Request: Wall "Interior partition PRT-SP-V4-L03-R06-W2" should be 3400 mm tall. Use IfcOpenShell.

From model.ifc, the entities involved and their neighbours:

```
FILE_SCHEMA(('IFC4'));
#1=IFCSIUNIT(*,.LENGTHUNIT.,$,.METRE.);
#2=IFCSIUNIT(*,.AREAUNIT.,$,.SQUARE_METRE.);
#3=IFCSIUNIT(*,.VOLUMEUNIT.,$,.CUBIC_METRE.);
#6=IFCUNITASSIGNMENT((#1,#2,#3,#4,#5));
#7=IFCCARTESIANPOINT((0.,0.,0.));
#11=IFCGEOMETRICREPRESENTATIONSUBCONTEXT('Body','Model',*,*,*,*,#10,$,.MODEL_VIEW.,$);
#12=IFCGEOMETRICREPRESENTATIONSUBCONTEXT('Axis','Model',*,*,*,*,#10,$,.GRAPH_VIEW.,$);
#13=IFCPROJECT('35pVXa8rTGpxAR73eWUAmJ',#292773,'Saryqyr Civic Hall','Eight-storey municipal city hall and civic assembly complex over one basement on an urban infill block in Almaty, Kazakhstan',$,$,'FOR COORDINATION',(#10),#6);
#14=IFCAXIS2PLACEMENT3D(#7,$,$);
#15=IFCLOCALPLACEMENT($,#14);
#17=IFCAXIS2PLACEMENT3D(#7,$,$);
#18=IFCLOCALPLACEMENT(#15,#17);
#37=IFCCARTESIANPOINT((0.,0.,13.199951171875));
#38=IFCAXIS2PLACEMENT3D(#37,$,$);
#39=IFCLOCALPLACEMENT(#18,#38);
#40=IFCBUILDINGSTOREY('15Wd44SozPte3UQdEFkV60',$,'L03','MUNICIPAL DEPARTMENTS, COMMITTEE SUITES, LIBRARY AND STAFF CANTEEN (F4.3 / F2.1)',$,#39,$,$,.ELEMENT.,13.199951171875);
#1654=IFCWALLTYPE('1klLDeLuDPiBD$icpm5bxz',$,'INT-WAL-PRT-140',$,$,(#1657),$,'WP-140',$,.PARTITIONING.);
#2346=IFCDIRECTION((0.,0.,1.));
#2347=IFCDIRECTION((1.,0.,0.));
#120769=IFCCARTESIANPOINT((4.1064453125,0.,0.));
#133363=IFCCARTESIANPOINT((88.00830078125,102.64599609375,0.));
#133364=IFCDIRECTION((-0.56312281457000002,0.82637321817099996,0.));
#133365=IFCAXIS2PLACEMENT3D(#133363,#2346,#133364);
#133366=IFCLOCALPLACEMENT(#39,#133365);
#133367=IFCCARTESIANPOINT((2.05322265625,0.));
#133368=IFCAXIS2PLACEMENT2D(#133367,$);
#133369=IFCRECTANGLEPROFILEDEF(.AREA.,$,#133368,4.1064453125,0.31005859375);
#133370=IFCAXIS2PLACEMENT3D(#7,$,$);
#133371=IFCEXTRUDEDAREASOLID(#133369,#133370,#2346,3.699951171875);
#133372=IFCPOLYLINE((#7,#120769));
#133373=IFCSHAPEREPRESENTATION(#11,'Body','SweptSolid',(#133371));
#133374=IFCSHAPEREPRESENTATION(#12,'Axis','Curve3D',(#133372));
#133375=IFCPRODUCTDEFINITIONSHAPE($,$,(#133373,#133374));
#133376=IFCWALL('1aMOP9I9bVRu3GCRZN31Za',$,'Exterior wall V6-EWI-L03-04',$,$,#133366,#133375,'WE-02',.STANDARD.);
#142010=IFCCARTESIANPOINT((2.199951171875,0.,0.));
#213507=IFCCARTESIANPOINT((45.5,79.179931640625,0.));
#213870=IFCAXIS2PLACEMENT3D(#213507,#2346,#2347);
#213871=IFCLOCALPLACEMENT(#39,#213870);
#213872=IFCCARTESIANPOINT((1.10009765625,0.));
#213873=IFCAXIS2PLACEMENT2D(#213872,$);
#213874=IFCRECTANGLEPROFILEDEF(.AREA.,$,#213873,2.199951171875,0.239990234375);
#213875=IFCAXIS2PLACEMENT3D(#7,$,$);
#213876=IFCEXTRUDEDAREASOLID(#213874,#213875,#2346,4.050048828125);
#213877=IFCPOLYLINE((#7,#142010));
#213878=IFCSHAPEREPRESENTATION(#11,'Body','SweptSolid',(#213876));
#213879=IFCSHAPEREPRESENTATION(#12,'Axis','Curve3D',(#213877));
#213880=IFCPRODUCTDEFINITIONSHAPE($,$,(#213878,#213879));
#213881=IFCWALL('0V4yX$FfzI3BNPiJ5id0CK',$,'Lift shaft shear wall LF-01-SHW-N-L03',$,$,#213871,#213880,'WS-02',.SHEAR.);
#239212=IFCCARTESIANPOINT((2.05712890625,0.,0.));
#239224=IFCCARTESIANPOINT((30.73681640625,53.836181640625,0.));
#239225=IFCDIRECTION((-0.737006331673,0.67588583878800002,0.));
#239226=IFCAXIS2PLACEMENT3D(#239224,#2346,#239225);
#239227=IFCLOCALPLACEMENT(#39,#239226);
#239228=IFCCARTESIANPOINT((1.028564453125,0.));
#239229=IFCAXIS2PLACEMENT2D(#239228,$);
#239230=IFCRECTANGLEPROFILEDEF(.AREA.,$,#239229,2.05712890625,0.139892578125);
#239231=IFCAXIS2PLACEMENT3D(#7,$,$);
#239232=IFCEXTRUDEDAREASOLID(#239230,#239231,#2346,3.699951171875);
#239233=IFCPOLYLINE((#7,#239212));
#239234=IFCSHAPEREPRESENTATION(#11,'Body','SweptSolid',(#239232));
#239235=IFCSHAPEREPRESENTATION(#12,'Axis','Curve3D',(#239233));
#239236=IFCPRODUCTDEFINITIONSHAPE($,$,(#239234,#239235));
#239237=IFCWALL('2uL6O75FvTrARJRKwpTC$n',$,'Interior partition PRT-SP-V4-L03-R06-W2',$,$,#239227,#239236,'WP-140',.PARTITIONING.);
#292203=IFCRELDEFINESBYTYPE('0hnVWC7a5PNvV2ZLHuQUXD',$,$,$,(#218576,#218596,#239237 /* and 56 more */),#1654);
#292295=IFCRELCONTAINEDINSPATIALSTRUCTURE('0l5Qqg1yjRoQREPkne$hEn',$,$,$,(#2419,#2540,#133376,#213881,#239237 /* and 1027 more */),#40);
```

```python
import ifcopenshell
import ifcopenshell.geom
import ifcopenshell.util.representation
import ifcopenshell.util.shape
import ifcopenshell.util.unit

model = ifcopenshell.open("model.ifc")
unit_scale = ifcopenshell.util.unit.calculate_unit_scale(model)
settings = ifcopenshell.geom.settings()


def volume(element):
    """Net volume in cubic metres, openings subtracted."""
    shape = ifcopenshell.geom.create_shape(settings, element)
    return ifcopenshell.util.shape.get_volume(shape.geometry)


wall = model.by_guid("2uL6O75FvTrARJRKwpTC$n")
before = volume(wall)

body = ifcopenshell.util.representation.get_representation(wall, "Model", "Body")
solid = body.Items[0]
old_height = solid.Depth
solid.Depth = 3.4 / unit_scale
after = volume(wall)

print(f"height {old_height:g} -> {solid.Depth:g}, volume {before:.3f} -> {after:.3f} m3")

model.write("model_edited.ifc")
```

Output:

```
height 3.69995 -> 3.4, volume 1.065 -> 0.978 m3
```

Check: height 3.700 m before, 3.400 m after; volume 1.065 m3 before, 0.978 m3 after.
